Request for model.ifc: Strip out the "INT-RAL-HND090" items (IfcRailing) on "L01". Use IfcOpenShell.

First a look at what the model holds.

```python
import ifcopenshell
import ifcopenshell.util.element

model = ifcopenshell.open("model.ifc")
print(model.schema)
storey = next(s for s in model.by_type("IfcBuildingStorey") if s.Name == "L01")
railings = [e for e in ifcopenshell.util.element.get_decomposition(storey) if e.is_a("IfcRailing")]
seen = {}
for e in railings:
    element_type = ifcopenshell.util.element.get_type(e)
    name = element_type.Name if element_type not in (None, e) else None
    seen[name] = seen.get(name, 0) + 1
for name, count in sorted(seen.items(), key=str):
    print(count, "x", name)
```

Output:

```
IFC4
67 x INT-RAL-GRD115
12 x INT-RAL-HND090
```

```python
import ifcopenshell
import ifcopenshell.api.root
import ifcopenshell.util.element

model = ifcopenshell.open("model.ifc")

storey = next(s for s in model.by_type("IfcBuildingStorey") if s.Name == "L01")
railings = [e for e in ifcopenshell.util.element.get_decomposition(storey) if e.is_a("IfcRailing")]
targets = [e for e in railings if (t := ifcopenshell.util.element.get_type(e)) not in (None, e) and t.Name == "INT-RAL-HND090"]

for e in targets:
    ifcopenshell.api.root.remove_product(model, product=e)
print(len(targets), "removed")

model.write("model_v2.ifc")
```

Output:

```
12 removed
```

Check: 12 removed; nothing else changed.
